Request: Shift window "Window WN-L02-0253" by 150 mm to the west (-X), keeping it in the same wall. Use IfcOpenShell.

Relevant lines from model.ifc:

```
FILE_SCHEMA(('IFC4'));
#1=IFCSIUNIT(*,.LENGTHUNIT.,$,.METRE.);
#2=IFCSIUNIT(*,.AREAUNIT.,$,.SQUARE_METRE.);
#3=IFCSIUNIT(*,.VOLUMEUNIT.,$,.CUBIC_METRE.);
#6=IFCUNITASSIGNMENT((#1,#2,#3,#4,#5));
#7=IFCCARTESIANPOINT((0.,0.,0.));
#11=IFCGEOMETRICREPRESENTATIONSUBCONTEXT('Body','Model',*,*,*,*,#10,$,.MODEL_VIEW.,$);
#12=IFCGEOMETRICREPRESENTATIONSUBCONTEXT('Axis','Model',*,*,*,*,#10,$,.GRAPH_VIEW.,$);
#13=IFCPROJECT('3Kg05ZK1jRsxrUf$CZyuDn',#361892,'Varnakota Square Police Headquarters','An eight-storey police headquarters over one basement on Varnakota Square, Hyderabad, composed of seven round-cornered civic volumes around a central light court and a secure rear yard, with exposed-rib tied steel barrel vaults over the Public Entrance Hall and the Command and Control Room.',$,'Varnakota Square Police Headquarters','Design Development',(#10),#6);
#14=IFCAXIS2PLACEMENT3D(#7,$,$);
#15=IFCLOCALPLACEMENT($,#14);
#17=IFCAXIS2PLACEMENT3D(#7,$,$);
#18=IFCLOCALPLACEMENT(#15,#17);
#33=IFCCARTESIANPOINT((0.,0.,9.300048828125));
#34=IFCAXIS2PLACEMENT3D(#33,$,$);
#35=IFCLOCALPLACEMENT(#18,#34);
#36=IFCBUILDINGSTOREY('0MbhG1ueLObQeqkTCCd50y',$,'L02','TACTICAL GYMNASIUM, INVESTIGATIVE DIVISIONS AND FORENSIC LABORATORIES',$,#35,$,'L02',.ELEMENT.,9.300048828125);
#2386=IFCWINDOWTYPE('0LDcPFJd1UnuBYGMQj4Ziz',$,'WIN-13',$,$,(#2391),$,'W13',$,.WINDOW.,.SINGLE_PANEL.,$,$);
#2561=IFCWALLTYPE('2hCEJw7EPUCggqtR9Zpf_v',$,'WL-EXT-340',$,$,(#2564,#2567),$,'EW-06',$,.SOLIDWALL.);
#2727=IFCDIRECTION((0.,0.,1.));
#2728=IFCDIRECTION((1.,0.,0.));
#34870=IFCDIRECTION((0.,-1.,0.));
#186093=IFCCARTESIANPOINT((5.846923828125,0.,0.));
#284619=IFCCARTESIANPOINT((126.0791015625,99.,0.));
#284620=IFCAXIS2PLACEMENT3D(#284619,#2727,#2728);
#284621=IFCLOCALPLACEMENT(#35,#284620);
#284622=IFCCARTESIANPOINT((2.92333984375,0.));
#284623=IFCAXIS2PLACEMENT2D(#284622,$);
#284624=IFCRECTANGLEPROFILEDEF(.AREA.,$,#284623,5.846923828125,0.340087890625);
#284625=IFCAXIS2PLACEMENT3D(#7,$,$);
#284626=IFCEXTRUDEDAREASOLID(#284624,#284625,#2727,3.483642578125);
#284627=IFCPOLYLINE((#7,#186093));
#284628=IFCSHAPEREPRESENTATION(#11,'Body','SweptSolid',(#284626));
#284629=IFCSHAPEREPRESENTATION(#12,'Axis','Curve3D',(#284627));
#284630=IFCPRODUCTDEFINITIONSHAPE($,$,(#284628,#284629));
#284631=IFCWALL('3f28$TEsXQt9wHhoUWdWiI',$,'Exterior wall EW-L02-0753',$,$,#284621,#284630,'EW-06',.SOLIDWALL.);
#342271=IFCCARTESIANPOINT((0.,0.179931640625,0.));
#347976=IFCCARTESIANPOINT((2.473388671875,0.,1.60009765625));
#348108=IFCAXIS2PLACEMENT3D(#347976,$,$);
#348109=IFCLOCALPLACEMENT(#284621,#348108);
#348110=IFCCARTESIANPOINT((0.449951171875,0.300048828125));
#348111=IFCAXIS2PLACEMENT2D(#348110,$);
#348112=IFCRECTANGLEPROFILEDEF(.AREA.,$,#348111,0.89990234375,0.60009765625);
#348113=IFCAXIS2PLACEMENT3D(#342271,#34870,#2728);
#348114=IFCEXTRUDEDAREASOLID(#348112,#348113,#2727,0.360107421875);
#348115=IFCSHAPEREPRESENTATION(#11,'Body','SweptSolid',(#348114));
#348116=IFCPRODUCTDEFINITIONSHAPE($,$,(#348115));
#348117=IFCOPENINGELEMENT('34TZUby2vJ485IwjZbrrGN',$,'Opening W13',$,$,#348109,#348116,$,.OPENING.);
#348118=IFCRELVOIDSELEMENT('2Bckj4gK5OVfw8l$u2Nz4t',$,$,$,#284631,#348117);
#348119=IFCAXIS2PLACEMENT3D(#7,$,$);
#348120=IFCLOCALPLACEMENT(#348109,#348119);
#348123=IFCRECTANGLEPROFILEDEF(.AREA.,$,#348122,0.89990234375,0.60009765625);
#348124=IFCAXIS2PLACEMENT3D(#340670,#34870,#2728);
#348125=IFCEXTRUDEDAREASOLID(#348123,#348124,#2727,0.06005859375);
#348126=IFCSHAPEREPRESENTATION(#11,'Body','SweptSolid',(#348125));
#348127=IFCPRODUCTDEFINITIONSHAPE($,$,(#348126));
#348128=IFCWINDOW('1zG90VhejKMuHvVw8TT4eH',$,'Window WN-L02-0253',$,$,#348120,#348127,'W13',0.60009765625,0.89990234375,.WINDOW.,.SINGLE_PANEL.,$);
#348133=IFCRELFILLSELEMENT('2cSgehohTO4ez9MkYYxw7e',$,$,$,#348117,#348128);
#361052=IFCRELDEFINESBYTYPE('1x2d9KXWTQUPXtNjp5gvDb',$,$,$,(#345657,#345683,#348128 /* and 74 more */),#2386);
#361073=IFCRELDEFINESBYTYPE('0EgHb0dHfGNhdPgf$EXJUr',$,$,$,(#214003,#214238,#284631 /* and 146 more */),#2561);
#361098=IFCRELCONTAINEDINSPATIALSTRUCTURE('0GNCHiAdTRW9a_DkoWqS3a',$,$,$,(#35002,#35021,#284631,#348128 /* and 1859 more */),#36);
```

```python
import ifcopenshell
import ifcopenshell.api.geometry
import ifcopenshell.util.placement
import ifcopenshell.util.unit

model = ifcopenshell.open("model.ifc")
unit_scale = ifcopenshell.util.unit.calculate_unit_scale(model)

window = model.by_id(348128)
opening = window.FillsVoids[0].RelatingOpeningElement
wall = opening.VoidsElements[0].RelatingBuildingElement

wall_matrix = ifcopenshell.util.placement.get_local_placement(wall.ObjectPlacement)
shift = wall_matrix[:3, 0] * -0.15 / unit_scale
before = ifcopenshell.util.placement.get_local_placement(window.ObjectPlacement)[:3, 3].copy()

# The window is placed relative to its opening, so it follows when the opening moves.
matrix = ifcopenshell.util.placement.get_local_placement(opening.ObjectPlacement)
matrix[:3, 3] += shift
ifcopenshell.api.geometry.edit_object_placement(
    model, product=opening, matrix=matrix, is_si=False, should_transform_children=True
)

after = ifcopenshell.util.placement.get_local_placement(window.ObjectPlacement)[:3, 3]
print("window moved by", (after - before).round(3) + 0.0)

model.write("model_edited.ifc")
```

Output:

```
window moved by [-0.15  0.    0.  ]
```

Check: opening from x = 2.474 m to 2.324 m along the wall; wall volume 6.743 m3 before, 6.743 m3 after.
